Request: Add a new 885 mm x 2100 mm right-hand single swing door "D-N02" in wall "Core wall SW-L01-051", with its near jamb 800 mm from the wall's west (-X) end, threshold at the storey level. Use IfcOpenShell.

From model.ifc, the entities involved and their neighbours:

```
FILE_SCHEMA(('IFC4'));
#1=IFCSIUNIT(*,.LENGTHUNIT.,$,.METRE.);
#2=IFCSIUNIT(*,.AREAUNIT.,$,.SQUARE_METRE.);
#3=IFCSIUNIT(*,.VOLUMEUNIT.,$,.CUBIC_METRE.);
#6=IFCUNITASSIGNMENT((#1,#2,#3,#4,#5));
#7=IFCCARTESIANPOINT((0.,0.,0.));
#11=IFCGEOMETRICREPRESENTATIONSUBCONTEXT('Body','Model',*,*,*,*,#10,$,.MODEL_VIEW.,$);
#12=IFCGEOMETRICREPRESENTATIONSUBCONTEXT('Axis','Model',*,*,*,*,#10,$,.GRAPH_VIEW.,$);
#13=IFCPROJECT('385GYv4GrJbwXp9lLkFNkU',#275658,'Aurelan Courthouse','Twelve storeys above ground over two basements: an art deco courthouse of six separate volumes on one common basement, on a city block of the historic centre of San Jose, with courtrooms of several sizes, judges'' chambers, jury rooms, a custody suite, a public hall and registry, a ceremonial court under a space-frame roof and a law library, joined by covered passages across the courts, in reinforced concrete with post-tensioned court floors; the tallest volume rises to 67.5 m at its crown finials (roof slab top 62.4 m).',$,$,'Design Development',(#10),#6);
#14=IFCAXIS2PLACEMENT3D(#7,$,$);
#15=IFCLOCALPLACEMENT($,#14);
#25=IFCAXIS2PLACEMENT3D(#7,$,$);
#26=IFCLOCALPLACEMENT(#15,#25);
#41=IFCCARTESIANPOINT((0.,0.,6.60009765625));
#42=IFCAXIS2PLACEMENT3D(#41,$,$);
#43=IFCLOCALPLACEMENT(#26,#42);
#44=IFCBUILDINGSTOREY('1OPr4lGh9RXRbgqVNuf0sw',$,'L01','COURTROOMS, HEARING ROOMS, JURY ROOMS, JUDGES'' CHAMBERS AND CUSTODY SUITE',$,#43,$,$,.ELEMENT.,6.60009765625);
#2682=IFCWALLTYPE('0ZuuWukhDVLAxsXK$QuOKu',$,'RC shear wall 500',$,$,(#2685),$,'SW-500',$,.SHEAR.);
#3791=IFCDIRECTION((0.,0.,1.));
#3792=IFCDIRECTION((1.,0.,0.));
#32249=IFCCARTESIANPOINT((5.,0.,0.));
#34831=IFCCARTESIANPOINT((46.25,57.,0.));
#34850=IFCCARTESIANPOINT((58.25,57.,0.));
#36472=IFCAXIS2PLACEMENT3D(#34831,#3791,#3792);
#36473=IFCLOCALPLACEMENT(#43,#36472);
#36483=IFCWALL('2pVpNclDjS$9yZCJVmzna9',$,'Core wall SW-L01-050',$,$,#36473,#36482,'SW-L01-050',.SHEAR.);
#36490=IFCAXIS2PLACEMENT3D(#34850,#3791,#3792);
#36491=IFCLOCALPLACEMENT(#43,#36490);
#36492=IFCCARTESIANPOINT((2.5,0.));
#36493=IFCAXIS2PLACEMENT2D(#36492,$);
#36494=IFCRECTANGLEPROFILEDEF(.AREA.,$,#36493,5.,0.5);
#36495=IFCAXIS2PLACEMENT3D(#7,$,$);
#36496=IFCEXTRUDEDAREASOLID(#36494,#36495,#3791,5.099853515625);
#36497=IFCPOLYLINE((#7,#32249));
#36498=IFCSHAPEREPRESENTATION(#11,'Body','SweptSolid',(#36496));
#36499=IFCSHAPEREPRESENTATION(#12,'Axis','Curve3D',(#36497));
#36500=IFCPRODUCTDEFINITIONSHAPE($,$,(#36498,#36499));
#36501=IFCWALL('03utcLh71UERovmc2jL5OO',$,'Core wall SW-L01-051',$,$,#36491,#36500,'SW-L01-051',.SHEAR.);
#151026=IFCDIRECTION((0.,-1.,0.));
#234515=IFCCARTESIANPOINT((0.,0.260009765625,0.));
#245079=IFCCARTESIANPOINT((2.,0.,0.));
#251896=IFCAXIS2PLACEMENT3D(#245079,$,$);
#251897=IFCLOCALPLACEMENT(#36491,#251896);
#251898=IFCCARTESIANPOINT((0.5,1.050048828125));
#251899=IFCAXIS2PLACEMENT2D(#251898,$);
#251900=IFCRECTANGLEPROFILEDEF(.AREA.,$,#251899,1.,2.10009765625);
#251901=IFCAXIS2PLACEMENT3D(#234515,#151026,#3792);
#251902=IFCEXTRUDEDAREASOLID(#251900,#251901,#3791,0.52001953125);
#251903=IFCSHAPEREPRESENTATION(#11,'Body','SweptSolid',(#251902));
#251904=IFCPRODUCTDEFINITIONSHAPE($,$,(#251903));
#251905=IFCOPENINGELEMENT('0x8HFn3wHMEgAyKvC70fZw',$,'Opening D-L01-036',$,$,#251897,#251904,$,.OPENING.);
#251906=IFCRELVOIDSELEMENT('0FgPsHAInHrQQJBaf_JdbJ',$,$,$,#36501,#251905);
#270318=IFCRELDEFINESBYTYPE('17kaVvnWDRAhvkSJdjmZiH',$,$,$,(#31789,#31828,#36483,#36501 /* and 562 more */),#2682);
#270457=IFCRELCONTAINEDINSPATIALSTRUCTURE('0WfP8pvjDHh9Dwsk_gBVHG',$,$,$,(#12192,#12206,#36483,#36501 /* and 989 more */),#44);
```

```python
import numpy as np
import ifcopenshell
import ifcopenshell.api.feature
import ifcopenshell.api.geometry
import ifcopenshell.api.root
import ifcopenshell.api.spatial
import ifcopenshell.geom
import ifcopenshell.util.element
import ifcopenshell.util.placement
import ifcopenshell.util.representation
import ifcopenshell.util.shape
import ifcopenshell.util.unit

model = ifcopenshell.open("model.ifc")
unit_scale = ifcopenshell.util.unit.calculate_unit_scale(model)
settings = ifcopenshell.geom.settings()


def volume(element):
    """Net volume in cubic metres, openings subtracted."""
    shape = ifcopenshell.geom.create_shape(settings, element)
    return ifcopenshell.util.shape.get_volume(shape.geometry)


wall = model.by_guid("03utcLh71UERovmc2jL5OO")
storey = ifcopenshell.util.element.get_container(wall, ifc_class="IfcBuildingStorey")
context = ifcopenshell.util.representation.get_context(model, "Model", "Body", "MODEL_VIEW")
before = volume(wall)

width, height, from_end, sill = 0.885, 2.1, 0.8, 0.0  # metres

# The wall runs along its own X axis, and the end named is its -X end.
wall_shape = ifcopenshell.geom.create_shape(settings, wall)
x, y, z = ifcopenshell.util.shape.get_vertices(wall_shape.geometry).T
start = x.min() + from_end
face, thickness = float(y.min()), float(y.max() - y.min())
wall_matrix = ifcopenshell.util.placement.get_local_placement(wall.ObjectPlacement)
level = ifcopenshell.util.placement.get_local_placement(storey.ObjectPlacement)[2, 3]


def in_wall(x, y):
    """Placement at x, y metres in the wall's axes, at sill height."""
    matrix = wall_matrix.copy()
    matrix[:, 3] = wall_matrix @ np.array([x / unit_scale, y / unit_scale, 0.0, 1.0])
    matrix[2, 3] = level + sill / unit_scale
    return matrix


# Opening: a box that overshoots both wall faces by 50 mm.
opening = ifcopenshell.api.root.create_entity(model, ifc_class="IfcOpeningElement", predefined_type="OPENING")
box = ifcopenshell.api.geometry.add_wall_representation(
    model, context=context, length=width, height=height, thickness=thickness + 0.1
)
ifcopenshell.api.geometry.assign_representation(model, product=opening, representation=box)
ifcopenshell.api.geometry.edit_object_placement(model, product=opening, matrix=in_wall(start, face - 0.05), is_si=False)
ifcopenshell.api.feature.add_feature(model, feature=opening, element=wall)

door = ifcopenshell.api.root.create_entity(model, ifc_class="IfcDoor", name="D-N02", predefined_type="DOOR")
door.OverallWidth, door.OverallHeight = width / unit_scale, height / unit_scale
door.OperationType = "SINGLE_SWING_RIGHT"
body = ifcopenshell.api.geometry.add_door_representation(
    model,
    context=context,
    overall_width=door.OverallWidth,
    overall_height=door.OverallHeight,
    operation_type="SINGLE_SWING_RIGHT",
    lining_properties={"LiningDepth": thickness / unit_scale, "ThresholdDepth": thickness / unit_scale},
)
ifcopenshell.api.geometry.assign_representation(model, product=door, representation=body)
ifcopenshell.api.spatial.assign_container(model, products=[door], relating_structure=storey)
ifcopenshell.api.feature.add_filling(model, opening=opening, element=door)

# The lining spans the wall, so the door starts at the wall face.
ifcopenshell.api.geometry.edit_object_placement(model, product=door, matrix=in_wall(start, face), is_si=False)

after = volume(wall)

print(f"wall volume {before:.3f} -> {after:.3f} m3")

model.write("model_updated.ifc")
```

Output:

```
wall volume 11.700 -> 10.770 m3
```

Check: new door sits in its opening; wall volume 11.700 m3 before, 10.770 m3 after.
